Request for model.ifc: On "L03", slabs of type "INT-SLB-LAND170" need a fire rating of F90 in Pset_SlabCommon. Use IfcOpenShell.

First a look at what the model holds.

```python
import ifcopenshell
import ifcopenshell.util.element

model = ifcopenshell.open("model.ifc")
print(model.schema)
storey = next(s for s in model.by_type("IfcBuildingStorey") if s.Name == "L03")
slabs = [e for e in ifcopenshell.util.element.get_decomposition(storey) if e.is_a("IfcSlab")]
seen = {}
for e in slabs:
    element_type = ifcopenshell.util.element.get_type(e)
    key = (element_type.Name if element_type != e and element_type else None, ifcopenshell.util.element.get_pset(e, "Pset_SlabCommon", "FireRating"))
    seen[key] = seen.get(key, 0) + 1
for (name, value), count in sorted(seen.items(), key=str):
    print(count, "x", name, "|", value)
```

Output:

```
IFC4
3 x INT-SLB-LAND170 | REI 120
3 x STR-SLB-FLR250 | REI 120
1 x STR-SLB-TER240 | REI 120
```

```python
import ifcopenshell
import ifcopenshell.api.pset
import ifcopenshell.util.element

model = ifcopenshell.open("model.ifc")

storey = next(s for s in model.by_type("IfcBuildingStorey") if s.Name == "L03")
slabs = [e for e in ifcopenshell.util.element.get_decomposition(storey) if e.is_a("IfcSlab")]

count = 0
for e in slabs:
    element_type = ifcopenshell.util.element.get_type(e)
    if element_type in (None, e) or element_type.Name != "INT-SLB-LAND170":
        continue
    # add_pset returns the element's existing set when there is one.
    pset = ifcopenshell.api.pset.add_pset(model, product=e, name="Pset_SlabCommon")
    ifcopenshell.api.pset.edit_pset(model, pset=pset, properties={"FireRating": "F90"})
    count += 1

print(count, "slabs updated")

model.write("model_v2.ifc")
```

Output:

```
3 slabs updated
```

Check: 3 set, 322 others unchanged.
